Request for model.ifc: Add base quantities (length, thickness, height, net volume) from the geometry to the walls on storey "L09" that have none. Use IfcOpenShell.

First a look at what the model holds.

```python
import ifcopenshell
import ifcopenshell.util.element
import ifcopenshell.util.unit

model = ifcopenshell.open("model.ifc")
print(model.schema)
for unit_type in ("LENGTHUNIT", "AREAUNIT", "VOLUMEUNIT"):
    print(unit_type, ifcopenshell.util.unit.calculate_unit_scale(model, unit_type))
storey = next(s for s in model.by_type("IfcBuildingStorey") if s.Name == "L09")
walls = [e for e in ifcopenshell.util.element.get_decomposition(storey) if e.is_a("IfcWall")]
for e in sorted(walls, key=lambda e: e.id()):
    print(e.id(), e.is_a(), e.Name, list(ifcopenshell.util.element.get_psets(e, qtos_only=True)), sep=" | ")
```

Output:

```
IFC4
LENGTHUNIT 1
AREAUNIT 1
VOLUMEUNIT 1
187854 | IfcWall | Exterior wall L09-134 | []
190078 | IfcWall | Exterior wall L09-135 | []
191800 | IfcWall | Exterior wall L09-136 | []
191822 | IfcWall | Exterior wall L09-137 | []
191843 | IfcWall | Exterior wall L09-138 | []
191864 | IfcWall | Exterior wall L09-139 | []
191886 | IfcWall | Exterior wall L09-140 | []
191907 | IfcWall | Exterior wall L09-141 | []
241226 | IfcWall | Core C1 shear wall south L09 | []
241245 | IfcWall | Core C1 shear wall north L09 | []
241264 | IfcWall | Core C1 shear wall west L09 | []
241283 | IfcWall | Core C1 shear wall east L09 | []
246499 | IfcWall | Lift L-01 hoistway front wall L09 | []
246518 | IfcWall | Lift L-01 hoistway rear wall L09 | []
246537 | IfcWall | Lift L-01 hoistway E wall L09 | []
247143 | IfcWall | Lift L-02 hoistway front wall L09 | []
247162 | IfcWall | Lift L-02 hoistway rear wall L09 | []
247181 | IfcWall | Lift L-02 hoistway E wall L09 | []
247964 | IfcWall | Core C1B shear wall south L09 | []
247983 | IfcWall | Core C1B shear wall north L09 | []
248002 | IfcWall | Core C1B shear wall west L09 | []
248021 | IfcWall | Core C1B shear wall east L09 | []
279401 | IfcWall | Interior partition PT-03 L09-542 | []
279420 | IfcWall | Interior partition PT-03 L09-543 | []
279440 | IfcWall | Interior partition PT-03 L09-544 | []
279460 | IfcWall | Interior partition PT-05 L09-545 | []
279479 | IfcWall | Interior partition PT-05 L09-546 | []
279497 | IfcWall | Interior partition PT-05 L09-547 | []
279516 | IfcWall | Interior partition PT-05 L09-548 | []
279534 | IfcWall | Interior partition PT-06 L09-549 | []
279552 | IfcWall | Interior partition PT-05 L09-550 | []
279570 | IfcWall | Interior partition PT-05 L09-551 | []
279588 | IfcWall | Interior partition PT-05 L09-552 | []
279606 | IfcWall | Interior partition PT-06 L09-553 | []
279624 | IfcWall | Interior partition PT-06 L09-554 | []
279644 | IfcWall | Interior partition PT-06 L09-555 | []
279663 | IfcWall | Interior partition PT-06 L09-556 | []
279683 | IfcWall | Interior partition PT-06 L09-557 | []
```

```python
import ifcopenshell
import ifcopenshell.api.pset
import ifcopenshell.geom
import ifcopenshell.util.element
import ifcopenshell.util.shape
import ifcopenshell.util.unit

model = ifcopenshell.open("model.ifc")
unit_scale = ifcopenshell.util.unit.calculate_unit_scale(model)
volume_scale = ifcopenshell.util.unit.calculate_unit_scale(model, "VOLUMEUNIT")
settings = ifcopenshell.geom.settings()

storey = next(s for s in model.by_type("IfcBuildingStorey") if s.Name == "L09")
walls = [e for e in ifcopenshell.util.element.get_decomposition(storey) if e.is_a("IfcWall")]

for e in sorted(walls, key=lambda e: e.id()):
    if ifcopenshell.util.element.get_psets(e, qtos_only=True, should_inherit=False):
        continue
    # Geometry comes back in metres, in the element's own axes.
    shape = ifcopenshell.geom.create_shape(settings, e)
    values = {
        "Length": ifcopenshell.util.shape.get_x(shape.geometry) / unit_scale,
        "Width": ifcopenshell.util.shape.get_y(shape.geometry) / unit_scale,
        "Height": ifcopenshell.util.shape.get_z(shape.geometry) / unit_scale,
        "NetVolume": ifcopenshell.util.shape.get_volume(shape.geometry) / volume_scale,
    }
    qto = ifcopenshell.api.pset.add_qto(model, product=e, name="Qto_WallBaseQuantities")
    ifcopenshell.api.pset.edit_qto(model, qto=qto, properties=values)
    print(e.id(), {k: round(v, 3) for k, v in values.items()})

model.write("model_updated.ifc")
```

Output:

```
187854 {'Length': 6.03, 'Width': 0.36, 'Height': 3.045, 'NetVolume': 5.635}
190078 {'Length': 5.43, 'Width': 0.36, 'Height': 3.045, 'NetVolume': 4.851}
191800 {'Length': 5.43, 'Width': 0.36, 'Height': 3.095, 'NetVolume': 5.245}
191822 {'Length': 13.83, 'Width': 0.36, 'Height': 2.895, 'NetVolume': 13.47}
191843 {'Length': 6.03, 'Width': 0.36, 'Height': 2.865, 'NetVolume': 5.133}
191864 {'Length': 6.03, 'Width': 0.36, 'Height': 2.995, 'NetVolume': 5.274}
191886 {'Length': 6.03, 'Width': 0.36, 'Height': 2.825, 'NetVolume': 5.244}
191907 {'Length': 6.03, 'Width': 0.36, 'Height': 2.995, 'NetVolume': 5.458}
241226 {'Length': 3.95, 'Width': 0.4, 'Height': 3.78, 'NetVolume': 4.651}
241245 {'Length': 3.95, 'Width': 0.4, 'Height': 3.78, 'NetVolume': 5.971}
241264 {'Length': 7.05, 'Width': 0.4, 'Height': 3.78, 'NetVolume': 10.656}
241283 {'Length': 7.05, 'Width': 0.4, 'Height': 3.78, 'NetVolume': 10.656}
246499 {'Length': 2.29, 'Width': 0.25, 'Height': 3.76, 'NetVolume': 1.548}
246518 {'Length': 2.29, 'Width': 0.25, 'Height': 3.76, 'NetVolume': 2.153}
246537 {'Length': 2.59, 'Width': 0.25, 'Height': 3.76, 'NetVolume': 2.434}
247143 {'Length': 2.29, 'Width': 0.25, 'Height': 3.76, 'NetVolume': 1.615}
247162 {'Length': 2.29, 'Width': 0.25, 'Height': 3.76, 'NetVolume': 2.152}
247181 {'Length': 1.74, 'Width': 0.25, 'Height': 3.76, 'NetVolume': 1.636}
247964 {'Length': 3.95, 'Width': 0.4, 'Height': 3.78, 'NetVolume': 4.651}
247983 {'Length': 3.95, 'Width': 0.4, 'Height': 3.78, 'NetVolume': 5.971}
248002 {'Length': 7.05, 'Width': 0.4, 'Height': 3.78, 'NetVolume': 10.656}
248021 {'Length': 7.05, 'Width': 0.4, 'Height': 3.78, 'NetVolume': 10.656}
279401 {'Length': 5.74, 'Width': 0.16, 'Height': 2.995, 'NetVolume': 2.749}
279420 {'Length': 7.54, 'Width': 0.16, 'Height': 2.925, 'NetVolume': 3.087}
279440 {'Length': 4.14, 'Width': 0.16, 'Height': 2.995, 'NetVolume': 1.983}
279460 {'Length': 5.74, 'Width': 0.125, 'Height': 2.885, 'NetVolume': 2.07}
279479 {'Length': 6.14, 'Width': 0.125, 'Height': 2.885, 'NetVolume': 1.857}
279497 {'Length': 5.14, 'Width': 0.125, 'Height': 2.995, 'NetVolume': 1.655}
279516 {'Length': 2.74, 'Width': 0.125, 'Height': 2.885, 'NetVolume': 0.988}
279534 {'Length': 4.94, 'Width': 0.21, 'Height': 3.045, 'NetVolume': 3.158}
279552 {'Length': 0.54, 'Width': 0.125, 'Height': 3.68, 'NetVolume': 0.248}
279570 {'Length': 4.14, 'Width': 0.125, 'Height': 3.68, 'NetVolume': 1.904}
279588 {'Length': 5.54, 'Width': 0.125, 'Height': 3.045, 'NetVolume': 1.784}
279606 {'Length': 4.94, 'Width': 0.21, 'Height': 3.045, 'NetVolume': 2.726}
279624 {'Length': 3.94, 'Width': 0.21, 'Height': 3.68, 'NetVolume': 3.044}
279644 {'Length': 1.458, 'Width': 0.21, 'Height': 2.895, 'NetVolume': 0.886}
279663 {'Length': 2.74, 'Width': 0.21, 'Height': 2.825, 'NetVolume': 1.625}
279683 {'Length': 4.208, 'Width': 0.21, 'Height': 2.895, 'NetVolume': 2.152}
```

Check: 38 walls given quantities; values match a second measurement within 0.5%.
